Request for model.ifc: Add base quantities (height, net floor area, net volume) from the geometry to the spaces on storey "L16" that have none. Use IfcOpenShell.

First a look at what the model holds.

```python
import ifcopenshell
import ifcopenshell.util.element
import ifcopenshell.util.unit

model = ifcopenshell.open("model.ifc")
print(model.schema)
for unit_type in ("LENGTHUNIT", "AREAUNIT", "VOLUMEUNIT"):
    print(unit_type, ifcopenshell.util.unit.calculate_unit_scale(model, unit_type))
storey = next(s for s in model.by_type("IfcBuildingStorey") if s.Name == "L16")
spaces = [e for e in ifcopenshell.util.element.get_decomposition(storey) if e.is_a("IfcSpace")]
for e in sorted(spaces, key=lambda e: e.id()):
    print(e.id(), e.is_a(), e.Name, list(ifcopenshell.util.element.get_psets(e, qtos_only=True)), sep=" | ")
```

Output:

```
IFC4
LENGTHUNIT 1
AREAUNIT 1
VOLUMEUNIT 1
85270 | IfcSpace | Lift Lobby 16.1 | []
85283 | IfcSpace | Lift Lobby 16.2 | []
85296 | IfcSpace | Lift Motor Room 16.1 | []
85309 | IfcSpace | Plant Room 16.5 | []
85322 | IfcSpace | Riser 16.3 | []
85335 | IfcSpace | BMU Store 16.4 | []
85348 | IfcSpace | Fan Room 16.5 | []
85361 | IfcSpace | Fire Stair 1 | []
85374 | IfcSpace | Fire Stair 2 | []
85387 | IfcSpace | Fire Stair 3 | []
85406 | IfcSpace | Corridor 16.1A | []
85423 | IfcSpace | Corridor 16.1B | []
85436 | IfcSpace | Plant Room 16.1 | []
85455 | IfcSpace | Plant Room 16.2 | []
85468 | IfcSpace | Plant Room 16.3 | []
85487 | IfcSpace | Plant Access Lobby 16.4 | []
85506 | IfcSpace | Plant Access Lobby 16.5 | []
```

```python
import ifcopenshell
import ifcopenshell.api.pset
import ifcopenshell.geom
import ifcopenshell.util.element
import ifcopenshell.util.shape
import ifcopenshell.util.unit

model = ifcopenshell.open("model.ifc")
unit_scale = ifcopenshell.util.unit.calculate_unit_scale(model)
area_scale = ifcopenshell.util.unit.calculate_unit_scale(model, "AREAUNIT")
volume_scale = ifcopenshell.util.unit.calculate_unit_scale(model, "VOLUMEUNIT")
settings = ifcopenshell.geom.settings()

storey = next(s for s in model.by_type("IfcBuildingStorey") if s.Name == "L16")
spaces = [e for e in ifcopenshell.util.element.get_decomposition(storey) if e.is_a("IfcSpace")]

for e in sorted(spaces, key=lambda e: e.id()):
    if ifcopenshell.util.element.get_psets(e, qtos_only=True, should_inherit=False):
        continue
    # Geometry comes back in metres, in the element's own axes.
    shape = ifcopenshell.geom.create_shape(settings, e)
    values = {
        "Height": ifcopenshell.util.shape.get_z(shape.geometry) / unit_scale,
        "NetFloorArea": ifcopenshell.util.shape.get_footprint_area(shape.geometry) / area_scale,
        "NetVolume": ifcopenshell.util.shape.get_volume(shape.geometry) / volume_scale,
    }
    qto = ifcopenshell.api.pset.add_qto(model, product=e, name="Qto_SpaceBaseQuantities")
    ifcopenshell.api.pset.edit_qto(model, qto=qto, properties=values)
    print(e.id(), {k: round(v, 3) for k, v in values.items()})

model.write("model_edited.ifc")
```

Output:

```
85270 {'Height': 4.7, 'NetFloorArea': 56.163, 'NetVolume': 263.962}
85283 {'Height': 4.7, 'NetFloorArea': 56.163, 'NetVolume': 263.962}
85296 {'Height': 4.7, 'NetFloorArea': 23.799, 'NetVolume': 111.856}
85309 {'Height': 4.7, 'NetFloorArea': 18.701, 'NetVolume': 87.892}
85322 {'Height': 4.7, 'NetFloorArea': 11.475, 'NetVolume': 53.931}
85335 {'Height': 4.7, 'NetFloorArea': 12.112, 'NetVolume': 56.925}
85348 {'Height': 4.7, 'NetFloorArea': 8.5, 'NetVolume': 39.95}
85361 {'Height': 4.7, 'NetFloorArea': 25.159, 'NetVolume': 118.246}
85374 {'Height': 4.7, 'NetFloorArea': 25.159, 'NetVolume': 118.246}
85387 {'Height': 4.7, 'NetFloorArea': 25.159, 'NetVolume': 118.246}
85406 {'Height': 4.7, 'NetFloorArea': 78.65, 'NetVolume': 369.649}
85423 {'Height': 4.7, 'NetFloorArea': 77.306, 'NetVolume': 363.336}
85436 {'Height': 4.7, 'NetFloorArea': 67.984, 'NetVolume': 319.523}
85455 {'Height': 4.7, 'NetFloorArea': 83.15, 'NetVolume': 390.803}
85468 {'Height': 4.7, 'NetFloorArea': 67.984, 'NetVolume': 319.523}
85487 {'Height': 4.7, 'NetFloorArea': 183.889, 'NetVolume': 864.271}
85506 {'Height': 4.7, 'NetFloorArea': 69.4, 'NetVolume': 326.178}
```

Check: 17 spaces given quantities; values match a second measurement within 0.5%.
